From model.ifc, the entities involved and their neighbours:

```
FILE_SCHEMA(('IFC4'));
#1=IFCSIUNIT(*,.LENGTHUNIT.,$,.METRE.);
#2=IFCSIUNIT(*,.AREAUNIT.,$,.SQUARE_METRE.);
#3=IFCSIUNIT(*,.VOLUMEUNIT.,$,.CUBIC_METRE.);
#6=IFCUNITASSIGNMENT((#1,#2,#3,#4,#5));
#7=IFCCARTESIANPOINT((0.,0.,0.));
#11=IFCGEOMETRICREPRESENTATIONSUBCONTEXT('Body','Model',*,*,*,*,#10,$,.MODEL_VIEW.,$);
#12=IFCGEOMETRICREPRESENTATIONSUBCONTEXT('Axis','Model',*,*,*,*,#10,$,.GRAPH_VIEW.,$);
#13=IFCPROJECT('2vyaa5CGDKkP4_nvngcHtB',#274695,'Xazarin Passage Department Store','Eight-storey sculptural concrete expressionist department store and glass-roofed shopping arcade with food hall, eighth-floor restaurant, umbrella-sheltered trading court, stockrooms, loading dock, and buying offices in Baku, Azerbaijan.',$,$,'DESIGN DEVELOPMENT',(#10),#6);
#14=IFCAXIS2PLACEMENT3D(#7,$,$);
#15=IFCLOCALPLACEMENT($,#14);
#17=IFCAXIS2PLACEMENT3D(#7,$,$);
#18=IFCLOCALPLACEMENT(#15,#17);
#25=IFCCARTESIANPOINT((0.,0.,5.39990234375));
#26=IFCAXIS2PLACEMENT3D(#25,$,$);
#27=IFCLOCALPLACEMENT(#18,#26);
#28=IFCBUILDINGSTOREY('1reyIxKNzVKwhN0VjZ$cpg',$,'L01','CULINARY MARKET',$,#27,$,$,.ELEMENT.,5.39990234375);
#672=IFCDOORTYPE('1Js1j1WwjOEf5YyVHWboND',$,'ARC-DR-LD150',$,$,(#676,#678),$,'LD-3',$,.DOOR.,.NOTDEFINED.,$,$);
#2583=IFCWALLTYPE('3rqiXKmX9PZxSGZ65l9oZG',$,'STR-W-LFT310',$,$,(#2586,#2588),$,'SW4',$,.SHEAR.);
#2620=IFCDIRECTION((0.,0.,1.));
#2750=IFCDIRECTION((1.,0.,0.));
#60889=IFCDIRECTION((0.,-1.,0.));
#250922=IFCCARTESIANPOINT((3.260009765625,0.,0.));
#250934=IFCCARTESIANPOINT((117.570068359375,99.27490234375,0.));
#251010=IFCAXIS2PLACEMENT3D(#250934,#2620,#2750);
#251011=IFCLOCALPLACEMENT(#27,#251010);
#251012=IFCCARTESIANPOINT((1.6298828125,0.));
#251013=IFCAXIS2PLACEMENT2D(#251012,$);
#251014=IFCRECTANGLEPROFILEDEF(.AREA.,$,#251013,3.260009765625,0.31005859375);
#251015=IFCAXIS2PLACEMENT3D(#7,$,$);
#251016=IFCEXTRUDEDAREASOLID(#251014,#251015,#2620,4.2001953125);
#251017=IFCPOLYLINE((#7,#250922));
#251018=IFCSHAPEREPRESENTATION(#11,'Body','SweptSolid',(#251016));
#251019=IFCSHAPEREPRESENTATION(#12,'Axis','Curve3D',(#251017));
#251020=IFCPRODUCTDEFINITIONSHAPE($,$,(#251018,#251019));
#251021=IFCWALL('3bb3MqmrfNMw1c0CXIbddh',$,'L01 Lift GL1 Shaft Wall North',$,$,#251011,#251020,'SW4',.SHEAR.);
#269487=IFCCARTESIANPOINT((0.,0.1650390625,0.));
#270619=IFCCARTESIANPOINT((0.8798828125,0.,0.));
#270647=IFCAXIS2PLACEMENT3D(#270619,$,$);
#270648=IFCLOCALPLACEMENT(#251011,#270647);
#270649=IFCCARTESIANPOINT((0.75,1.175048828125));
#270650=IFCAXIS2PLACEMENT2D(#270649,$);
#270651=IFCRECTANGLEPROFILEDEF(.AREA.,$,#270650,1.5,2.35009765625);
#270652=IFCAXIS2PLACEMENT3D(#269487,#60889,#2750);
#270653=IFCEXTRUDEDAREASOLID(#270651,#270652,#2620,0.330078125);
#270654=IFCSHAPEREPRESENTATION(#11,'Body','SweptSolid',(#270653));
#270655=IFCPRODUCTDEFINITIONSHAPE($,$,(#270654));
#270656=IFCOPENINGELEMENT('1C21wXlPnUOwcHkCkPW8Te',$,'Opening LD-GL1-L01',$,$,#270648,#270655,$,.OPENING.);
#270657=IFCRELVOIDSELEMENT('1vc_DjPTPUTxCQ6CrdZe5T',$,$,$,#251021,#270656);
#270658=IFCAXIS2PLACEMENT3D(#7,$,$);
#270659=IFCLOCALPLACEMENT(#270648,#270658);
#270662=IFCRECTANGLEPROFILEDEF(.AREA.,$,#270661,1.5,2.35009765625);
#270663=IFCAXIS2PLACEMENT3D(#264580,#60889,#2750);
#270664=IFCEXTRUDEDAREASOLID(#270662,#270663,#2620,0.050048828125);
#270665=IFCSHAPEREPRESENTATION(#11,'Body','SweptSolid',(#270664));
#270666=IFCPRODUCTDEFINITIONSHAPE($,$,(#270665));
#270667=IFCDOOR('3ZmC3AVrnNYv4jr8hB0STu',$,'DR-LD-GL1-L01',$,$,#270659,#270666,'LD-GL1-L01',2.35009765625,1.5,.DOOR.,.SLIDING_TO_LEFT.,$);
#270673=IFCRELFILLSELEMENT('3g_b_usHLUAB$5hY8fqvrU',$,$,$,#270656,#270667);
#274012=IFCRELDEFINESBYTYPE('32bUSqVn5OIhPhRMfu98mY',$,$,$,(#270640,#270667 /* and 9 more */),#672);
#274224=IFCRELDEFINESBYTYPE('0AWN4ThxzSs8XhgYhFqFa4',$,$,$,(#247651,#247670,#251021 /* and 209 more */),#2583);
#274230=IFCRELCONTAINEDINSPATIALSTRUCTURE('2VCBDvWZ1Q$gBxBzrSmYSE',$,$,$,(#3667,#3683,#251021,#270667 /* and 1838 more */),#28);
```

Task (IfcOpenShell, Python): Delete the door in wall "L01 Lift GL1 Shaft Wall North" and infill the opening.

```python
import ifcopenshell
import ifcopenshell.api.feature
import ifcopenshell.api.root
import ifcopenshell.geom
import ifcopenshell.util.shape

model = ifcopenshell.open("model.ifc")
settings = ifcopenshell.geom.settings()


def volume(element):
    """Net volume in cubic metres, openings subtracted."""
    shape = ifcopenshell.geom.create_shape(settings, element)
    return ifcopenshell.util.shape.get_volume(shape.geometry)


door = model.by_guid("3ZmC3AVrnNYv4jr8hB0STu")
opening = door.FillsVoids[0].RelatingOpeningElement
wall = opening.VoidsElements[0].RelatingBuildingElement
before = volume(wall)

ifcopenshell.api.root.remove_product(model, product=door)
ifcopenshell.api.feature.remove_feature(model, feature=opening)

after = volume(wall)

print(f"wall volume {before:.3f} -> {after:.3f} m3")

model.write("model_v2.ifc")
```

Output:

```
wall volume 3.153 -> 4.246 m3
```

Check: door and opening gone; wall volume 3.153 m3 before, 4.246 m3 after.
